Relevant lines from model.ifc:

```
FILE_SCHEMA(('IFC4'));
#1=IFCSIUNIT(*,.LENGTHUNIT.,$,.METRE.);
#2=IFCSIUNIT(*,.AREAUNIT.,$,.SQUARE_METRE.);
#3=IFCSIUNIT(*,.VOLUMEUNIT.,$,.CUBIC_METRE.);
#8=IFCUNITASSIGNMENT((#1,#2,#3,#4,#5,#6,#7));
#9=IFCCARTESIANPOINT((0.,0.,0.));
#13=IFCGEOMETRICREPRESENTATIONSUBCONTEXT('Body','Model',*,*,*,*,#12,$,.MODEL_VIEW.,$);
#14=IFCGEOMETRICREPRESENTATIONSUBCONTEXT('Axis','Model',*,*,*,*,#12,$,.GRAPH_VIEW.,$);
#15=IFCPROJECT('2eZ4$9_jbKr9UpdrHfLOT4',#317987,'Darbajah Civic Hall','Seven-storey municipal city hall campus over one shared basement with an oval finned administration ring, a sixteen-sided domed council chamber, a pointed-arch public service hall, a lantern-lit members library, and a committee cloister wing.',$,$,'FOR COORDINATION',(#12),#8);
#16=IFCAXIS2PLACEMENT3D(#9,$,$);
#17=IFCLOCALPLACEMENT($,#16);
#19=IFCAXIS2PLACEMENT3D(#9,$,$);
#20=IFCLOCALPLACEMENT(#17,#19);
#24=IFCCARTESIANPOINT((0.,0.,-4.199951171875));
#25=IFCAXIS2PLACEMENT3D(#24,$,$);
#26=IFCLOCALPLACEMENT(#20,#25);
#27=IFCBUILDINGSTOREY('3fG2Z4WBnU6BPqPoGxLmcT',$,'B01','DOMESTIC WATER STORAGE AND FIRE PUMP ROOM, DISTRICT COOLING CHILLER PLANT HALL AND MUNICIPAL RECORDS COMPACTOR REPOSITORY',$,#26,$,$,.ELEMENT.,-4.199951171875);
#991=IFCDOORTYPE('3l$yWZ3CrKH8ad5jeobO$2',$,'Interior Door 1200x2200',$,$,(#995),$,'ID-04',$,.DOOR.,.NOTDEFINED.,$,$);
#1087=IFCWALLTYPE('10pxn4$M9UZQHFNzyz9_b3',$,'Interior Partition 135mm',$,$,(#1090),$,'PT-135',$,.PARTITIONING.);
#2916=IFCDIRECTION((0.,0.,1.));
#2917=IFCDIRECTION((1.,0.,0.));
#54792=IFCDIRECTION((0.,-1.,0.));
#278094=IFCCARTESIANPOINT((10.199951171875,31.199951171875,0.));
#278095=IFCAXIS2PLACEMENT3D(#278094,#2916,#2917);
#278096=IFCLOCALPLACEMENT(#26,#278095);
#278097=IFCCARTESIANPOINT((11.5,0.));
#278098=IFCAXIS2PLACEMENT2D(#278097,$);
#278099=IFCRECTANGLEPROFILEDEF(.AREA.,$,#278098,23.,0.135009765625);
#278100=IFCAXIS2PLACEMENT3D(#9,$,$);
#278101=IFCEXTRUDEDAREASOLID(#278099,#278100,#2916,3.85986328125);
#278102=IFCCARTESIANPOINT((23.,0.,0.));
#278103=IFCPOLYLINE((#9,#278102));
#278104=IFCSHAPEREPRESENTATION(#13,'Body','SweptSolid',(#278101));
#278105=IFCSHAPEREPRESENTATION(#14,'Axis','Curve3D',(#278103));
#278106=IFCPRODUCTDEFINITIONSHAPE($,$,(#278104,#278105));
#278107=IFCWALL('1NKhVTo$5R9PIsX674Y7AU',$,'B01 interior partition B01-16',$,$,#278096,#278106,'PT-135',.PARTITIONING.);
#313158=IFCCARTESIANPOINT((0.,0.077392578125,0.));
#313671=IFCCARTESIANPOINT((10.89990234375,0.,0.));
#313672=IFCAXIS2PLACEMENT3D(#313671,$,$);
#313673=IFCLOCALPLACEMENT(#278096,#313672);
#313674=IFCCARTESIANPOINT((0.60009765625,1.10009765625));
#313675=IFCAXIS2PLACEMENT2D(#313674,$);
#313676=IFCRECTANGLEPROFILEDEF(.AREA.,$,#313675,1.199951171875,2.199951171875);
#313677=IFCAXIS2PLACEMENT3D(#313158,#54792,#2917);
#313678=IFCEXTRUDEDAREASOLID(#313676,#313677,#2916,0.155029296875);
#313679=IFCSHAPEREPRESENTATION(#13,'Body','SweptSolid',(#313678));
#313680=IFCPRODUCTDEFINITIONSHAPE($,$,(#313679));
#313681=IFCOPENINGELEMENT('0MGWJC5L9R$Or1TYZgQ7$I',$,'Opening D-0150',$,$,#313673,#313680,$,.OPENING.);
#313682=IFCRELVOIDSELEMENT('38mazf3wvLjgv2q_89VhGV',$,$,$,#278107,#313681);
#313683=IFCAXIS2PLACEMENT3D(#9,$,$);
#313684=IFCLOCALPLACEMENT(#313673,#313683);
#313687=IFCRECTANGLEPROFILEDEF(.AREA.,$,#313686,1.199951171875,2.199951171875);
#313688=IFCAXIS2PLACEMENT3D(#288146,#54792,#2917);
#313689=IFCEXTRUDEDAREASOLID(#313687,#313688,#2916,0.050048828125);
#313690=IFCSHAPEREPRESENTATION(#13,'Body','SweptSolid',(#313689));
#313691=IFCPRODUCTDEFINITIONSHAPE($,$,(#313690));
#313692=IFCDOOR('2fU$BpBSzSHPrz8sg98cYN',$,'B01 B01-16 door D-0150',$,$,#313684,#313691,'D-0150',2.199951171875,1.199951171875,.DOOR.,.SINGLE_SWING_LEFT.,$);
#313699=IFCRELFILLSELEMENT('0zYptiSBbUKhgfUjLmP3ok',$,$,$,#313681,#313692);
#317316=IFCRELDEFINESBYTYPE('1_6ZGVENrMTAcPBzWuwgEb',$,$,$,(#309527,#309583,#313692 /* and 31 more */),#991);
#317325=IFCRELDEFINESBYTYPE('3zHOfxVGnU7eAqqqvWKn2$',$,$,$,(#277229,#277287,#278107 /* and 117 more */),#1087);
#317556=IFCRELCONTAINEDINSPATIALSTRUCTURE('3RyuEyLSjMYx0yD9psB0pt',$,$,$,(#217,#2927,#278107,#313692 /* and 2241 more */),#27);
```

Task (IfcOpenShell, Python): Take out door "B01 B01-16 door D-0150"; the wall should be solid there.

```python
import ifcopenshell
import ifcopenshell.api.feature
import ifcopenshell.api.root
import ifcopenshell.geom
import ifcopenshell.util.shape

model = ifcopenshell.open("model.ifc")
settings = ifcopenshell.geom.settings()


def volume(element):
    """Net volume in cubic metres, openings subtracted."""
    shape = ifcopenshell.geom.create_shape(settings, element)
    return ifcopenshell.util.shape.get_volume(shape.geometry)


door = model.by_guid("2fU$BpBSzSHPrz8sg98cYN")
opening = door.FillsVoids[0].RelatingOpeningElement
wall = opening.VoidsElements[0].RelatingBuildingElement
before = volume(wall)

ifcopenshell.api.root.remove_product(model, product=door)
ifcopenshell.api.feature.remove_feature(model, feature=opening)

after = volume(wall)

print(f"wall volume {before:.3f} -> {after:.3f} m3")

model.write("model-out.ifc")
```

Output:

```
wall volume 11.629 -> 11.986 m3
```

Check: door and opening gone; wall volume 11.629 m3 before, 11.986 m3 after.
